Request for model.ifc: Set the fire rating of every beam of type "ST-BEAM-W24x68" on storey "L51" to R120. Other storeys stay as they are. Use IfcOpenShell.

First a look at what the model holds.

```python
import ifcopenshell
import ifcopenshell.util.element

model = ifcopenshell.open("model.ifc")
print(model.schema)
storey = next(s for s in model.by_type("IfcBuildingStorey") if s.Name == "L51")
beams = [e for e in ifcopenshell.util.element.get_decomposition(storey) if e.is_a("IfcBeam")]
seen = {}
for e in beams:
    element_type = ifcopenshell.util.element.get_type(e)
    key = (element_type.Name if element_type != e and element_type else None, ifcopenshell.util.element.get_pset(e, "Pset_BeamCommon", "FireRating"))
    seen[key] = seen.get(key, 0) + 1
for (name, value), count in sorted(seen.items(), key=str):
    print(count, "x", name, "|", value)
```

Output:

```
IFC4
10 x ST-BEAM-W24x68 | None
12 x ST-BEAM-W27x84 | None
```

```python
import ifcopenshell
import ifcopenshell.api.pset
import ifcopenshell.util.element

model = ifcopenshell.open("model.ifc")

storey = next(s for s in model.by_type("IfcBuildingStorey") if s.Name == "L51")
beams = [e for e in ifcopenshell.util.element.get_decomposition(storey) if e.is_a("IfcBeam")]

count = 0
for e in beams:
    element_type = ifcopenshell.util.element.get_type(e)
    if element_type in (None, e) or element_type.Name != "ST-BEAM-W24x68":
        continue
    found = ifcopenshell.util.element.get_pset(e, "Pset_BeamCommon", should_inherit=False)
    if found:
        pset = model.by_id(found["id"])
        if len(ifcopenshell.util.element.get_elements_by_pset(pset)) > 1:
            pset = ifcopenshell.api.pset.unshare_pset(model, products=[e], pset=pset)[0]
    else:
        pset = ifcopenshell.api.pset.add_pset(model, product=e, name="Pset_BeamCommon")
    ifcopenshell.api.pset.edit_pset(model, pset=pset, properties={"FireRating": "R120"})
    count += 1

print(count, "beams updated")

model.write("model_v2.ifc")
```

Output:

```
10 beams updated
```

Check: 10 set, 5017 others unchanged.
